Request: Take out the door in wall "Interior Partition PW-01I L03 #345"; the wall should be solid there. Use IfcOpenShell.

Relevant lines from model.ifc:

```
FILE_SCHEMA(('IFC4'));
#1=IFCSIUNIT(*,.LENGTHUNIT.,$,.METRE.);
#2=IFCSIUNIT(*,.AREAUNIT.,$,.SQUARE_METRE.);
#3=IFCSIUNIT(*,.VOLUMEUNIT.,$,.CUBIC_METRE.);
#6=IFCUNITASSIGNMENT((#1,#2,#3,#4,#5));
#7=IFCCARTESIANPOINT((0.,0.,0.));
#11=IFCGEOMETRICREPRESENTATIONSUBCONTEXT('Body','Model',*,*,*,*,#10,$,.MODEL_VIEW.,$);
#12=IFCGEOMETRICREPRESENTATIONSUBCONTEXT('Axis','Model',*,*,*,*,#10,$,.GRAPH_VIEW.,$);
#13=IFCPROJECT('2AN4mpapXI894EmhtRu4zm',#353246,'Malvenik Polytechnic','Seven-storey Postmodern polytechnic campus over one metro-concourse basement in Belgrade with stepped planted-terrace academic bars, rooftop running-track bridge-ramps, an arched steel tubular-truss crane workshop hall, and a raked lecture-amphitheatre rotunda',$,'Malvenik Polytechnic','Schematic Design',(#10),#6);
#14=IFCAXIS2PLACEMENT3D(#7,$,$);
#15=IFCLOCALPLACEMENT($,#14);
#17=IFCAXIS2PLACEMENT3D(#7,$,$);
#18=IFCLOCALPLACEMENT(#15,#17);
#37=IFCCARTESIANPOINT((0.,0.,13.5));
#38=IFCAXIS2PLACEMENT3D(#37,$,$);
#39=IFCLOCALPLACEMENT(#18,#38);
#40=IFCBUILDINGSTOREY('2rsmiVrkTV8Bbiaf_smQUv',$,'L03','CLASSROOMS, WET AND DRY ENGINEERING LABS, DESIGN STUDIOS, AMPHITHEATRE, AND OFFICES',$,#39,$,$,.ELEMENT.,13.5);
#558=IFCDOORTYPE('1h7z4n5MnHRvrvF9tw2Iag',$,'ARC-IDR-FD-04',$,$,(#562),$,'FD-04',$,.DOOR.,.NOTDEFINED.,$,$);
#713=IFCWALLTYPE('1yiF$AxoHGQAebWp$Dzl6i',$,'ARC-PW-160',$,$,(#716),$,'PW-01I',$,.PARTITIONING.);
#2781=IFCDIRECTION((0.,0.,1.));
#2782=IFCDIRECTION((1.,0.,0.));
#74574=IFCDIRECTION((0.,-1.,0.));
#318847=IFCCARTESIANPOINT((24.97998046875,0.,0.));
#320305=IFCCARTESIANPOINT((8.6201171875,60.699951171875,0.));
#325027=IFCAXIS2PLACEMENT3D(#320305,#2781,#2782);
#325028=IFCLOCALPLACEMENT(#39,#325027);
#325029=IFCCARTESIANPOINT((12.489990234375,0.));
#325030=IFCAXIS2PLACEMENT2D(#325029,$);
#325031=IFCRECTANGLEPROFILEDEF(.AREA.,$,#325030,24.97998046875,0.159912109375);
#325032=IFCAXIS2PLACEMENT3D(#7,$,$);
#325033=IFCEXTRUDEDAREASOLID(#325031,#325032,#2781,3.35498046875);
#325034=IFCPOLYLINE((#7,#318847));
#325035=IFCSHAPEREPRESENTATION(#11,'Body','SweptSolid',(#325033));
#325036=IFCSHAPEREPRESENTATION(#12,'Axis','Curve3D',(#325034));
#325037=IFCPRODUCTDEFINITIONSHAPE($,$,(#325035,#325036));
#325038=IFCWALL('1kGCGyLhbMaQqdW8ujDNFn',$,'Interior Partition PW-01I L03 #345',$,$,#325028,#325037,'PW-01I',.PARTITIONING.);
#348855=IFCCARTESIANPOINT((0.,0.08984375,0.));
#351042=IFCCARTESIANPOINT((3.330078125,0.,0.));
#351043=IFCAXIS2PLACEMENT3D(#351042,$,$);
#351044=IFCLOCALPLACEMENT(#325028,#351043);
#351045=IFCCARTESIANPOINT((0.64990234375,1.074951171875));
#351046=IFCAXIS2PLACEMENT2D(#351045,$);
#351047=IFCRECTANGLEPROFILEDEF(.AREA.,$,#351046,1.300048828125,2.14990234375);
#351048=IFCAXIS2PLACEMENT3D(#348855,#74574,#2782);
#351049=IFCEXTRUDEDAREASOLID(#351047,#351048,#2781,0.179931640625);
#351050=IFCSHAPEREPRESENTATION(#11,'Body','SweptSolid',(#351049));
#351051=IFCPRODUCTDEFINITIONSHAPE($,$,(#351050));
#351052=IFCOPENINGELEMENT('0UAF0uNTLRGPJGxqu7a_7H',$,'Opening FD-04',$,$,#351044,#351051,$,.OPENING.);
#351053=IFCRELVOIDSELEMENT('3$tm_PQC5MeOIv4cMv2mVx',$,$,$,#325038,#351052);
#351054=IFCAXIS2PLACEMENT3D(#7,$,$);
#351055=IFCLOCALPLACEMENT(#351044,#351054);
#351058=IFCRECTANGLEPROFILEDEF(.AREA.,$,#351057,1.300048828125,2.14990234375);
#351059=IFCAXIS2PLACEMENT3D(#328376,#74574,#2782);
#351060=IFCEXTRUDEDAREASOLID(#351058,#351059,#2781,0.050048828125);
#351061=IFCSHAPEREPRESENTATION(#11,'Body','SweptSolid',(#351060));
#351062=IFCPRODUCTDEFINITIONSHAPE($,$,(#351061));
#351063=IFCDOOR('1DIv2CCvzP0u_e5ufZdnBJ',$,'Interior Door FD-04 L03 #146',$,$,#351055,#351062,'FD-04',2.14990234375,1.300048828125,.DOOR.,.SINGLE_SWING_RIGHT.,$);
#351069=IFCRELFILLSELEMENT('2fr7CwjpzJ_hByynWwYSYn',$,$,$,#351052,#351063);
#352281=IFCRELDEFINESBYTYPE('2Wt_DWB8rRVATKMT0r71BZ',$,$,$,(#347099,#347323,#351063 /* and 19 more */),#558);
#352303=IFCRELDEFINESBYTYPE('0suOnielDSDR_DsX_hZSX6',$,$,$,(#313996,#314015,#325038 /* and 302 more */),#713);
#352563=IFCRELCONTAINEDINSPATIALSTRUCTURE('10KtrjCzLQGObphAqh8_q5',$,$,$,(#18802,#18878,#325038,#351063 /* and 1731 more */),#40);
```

```python
import ifcopenshell
import ifcopenshell.api.feature
import ifcopenshell.api.root
import ifcopenshell.geom
import ifcopenshell.util.shape

model = ifcopenshell.open("model.ifc")
settings = ifcopenshell.geom.settings()


def volume(element):
    """Net volume in cubic metres, openings subtracted."""
    shape = ifcopenshell.geom.create_shape(settings, element)
    return ifcopenshell.util.shape.get_volume(shape.geometry)


door = model.by_id(351063)
opening = door.FillsVoids[0].RelatingOpeningElement
wall = opening.VoidsElements[0].RelatingBuildingElement
before = volume(wall)

ifcopenshell.api.root.remove_product(model, product=door)
ifcopenshell.api.feature.remove_feature(model, feature=opening)

after = volume(wall)

print(f"wall volume {before:.3f} -> {after:.3f} m3")

model.write("model_rev.ifc")
```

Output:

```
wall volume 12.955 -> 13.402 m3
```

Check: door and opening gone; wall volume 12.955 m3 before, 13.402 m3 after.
